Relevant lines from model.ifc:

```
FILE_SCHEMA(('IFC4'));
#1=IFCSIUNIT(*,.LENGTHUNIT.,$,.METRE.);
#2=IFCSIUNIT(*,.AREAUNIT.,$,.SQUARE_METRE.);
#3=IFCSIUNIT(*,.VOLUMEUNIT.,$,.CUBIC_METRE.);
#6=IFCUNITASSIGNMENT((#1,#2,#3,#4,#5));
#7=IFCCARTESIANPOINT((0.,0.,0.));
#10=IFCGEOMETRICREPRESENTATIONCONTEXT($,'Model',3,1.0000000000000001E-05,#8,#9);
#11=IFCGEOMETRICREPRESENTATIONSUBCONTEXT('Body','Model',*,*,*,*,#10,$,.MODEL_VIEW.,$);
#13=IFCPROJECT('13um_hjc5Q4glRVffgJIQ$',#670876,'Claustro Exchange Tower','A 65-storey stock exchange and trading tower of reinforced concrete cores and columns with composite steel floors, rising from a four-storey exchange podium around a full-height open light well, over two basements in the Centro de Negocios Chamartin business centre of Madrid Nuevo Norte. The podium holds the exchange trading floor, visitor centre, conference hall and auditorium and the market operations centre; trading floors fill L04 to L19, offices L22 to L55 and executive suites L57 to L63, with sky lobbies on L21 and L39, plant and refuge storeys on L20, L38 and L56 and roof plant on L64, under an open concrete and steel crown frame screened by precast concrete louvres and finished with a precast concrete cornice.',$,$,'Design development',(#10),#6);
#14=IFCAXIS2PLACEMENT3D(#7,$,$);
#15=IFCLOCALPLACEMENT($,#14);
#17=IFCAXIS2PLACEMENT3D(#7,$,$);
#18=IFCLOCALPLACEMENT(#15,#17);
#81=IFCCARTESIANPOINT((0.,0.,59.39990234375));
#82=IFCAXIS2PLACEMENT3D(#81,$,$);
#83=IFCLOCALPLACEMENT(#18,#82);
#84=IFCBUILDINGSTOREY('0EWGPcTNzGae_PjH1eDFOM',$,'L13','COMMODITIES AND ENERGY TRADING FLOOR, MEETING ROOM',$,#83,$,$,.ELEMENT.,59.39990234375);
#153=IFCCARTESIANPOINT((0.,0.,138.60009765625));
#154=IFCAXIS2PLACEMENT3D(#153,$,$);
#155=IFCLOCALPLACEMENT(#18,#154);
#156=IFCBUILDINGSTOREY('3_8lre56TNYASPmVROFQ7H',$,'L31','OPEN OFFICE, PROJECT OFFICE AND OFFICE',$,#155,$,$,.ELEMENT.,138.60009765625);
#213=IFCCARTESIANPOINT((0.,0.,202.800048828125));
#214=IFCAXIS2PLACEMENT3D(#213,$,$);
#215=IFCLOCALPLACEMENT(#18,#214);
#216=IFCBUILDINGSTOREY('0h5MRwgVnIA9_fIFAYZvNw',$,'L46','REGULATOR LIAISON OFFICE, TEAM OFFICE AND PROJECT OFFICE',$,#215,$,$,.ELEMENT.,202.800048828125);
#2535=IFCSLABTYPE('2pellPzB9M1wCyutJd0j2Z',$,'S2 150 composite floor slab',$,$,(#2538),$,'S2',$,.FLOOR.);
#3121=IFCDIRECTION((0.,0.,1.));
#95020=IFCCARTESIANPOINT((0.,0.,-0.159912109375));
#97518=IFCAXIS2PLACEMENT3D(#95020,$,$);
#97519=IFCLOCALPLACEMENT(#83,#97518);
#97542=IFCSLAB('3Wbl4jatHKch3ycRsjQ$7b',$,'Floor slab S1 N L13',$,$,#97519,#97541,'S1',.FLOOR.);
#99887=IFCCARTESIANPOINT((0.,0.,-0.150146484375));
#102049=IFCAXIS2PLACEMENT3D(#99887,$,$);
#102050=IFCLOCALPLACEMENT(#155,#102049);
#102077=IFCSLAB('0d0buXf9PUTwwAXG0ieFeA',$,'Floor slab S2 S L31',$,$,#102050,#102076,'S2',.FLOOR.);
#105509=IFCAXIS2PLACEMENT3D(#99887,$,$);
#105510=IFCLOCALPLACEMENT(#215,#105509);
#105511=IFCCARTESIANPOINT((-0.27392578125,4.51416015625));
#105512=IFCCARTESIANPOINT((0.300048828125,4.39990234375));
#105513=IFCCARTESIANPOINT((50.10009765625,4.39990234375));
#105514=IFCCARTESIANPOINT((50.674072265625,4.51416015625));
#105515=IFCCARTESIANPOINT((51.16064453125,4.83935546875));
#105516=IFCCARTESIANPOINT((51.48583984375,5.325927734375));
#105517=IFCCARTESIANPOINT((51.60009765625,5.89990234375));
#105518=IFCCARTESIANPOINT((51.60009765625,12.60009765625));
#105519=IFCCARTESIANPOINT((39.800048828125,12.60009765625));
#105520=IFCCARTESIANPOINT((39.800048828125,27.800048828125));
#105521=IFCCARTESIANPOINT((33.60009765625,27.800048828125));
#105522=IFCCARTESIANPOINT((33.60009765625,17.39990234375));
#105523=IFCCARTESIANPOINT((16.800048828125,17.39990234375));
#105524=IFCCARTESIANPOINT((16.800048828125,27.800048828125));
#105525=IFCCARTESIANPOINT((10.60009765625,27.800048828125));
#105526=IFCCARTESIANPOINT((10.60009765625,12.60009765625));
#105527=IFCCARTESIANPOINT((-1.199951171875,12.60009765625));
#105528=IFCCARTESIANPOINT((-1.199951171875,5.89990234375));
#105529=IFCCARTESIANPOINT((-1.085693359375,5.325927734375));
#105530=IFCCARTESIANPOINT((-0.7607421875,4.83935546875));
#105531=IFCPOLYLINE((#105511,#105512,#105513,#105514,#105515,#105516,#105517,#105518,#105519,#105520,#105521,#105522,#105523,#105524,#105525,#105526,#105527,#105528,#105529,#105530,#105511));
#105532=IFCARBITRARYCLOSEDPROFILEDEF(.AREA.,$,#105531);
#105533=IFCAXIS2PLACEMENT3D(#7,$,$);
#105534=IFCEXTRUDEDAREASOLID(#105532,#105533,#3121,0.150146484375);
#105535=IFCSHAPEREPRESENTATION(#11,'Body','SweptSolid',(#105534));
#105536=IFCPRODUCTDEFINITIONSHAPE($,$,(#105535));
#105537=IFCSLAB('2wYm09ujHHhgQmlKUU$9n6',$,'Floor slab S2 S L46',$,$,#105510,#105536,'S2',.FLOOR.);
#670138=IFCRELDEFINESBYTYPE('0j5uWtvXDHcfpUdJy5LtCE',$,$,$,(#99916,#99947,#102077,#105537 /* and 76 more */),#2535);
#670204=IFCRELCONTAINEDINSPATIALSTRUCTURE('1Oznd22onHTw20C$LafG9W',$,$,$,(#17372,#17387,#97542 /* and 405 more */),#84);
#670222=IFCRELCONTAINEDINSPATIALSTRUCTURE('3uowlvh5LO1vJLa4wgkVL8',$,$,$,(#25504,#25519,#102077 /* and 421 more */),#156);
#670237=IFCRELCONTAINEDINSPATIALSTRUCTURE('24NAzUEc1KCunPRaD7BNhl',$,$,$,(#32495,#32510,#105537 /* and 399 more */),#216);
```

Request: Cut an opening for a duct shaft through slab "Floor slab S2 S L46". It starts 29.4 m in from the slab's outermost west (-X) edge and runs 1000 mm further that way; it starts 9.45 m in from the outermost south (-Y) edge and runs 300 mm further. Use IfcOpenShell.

```python
import numpy as np
import ifcopenshell
import ifcopenshell.api.feature
import ifcopenshell.api.geometry
import ifcopenshell.api.root
import ifcopenshell.geom
import ifcopenshell.util.placement
import ifcopenshell.util.representation
import ifcopenshell.util.shape
import ifcopenshell.util.unit

model = ifcopenshell.open("model.ifc")
unit_scale = ifcopenshell.util.unit.calculate_unit_scale(model)
settings = ifcopenshell.geom.settings()


def volume(element):
    """Net volume in cubic metres, openings subtracted."""
    shape = ifcopenshell.geom.create_shape(settings, element)
    return ifcopenshell.util.shape.get_volume(shape.geometry)


slab = model.by_guid("2wYm09ujHHhgQmlKUU$9n6")
before = volume(slab)

# Extent in the slab's own axes, in metres. The edges named are its -X and -Y sides.
slab_shape = ifcopenshell.geom.create_shape(settings, slab)
vertices = ifcopenshell.util.shape.get_vertices(slab_shape.geometry)
x_min, y_min, bottom = vertices.min(axis=0)
top = vertices[:, 2].max()

opening = ifcopenshell.api.root.create_entity(model, ifc_class="IfcOpeningElement", name="Duct shaft opening", predefined_type="OPENING")
context = ifcopenshell.util.representation.get_context(model, "Model", "Body", "MODEL_VIEW")
width, depth = 1, 0.3
outline = [(0.0, 0.0), (width, 0.0), (width, depth), (0.0, depth), (0.0, 0.0)]
# Overshoot both faces by 50 mm so the cut is clean.
shape = ifcopenshell.api.geometry.add_slab_representation(
    model, context=context, depth=top - bottom + 0.1, polyline=outline
)
ifcopenshell.api.geometry.assign_representation(model, product=opening, representation=shape)

matrix = ifcopenshell.util.placement.get_local_placement(slab.ObjectPlacement)
matrix[:, 3] = matrix @ np.append(np.array([x_min + 29.4, y_min + 9.45, bottom - 0.05]) / unit_scale, 1.0)
ifcopenshell.api.geometry.edit_object_placement(model, product=opening, matrix=matrix, is_si=False)
ifcopenshell.api.feature.add_feature(model, feature=opening, element=slab)

after = volume(slab)

print(f"slab volume {before:.3f} -> {after:.3f} m3")

model.write("model_edited.ifc")
```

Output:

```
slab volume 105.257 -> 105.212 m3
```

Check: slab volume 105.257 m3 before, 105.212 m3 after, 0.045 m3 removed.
